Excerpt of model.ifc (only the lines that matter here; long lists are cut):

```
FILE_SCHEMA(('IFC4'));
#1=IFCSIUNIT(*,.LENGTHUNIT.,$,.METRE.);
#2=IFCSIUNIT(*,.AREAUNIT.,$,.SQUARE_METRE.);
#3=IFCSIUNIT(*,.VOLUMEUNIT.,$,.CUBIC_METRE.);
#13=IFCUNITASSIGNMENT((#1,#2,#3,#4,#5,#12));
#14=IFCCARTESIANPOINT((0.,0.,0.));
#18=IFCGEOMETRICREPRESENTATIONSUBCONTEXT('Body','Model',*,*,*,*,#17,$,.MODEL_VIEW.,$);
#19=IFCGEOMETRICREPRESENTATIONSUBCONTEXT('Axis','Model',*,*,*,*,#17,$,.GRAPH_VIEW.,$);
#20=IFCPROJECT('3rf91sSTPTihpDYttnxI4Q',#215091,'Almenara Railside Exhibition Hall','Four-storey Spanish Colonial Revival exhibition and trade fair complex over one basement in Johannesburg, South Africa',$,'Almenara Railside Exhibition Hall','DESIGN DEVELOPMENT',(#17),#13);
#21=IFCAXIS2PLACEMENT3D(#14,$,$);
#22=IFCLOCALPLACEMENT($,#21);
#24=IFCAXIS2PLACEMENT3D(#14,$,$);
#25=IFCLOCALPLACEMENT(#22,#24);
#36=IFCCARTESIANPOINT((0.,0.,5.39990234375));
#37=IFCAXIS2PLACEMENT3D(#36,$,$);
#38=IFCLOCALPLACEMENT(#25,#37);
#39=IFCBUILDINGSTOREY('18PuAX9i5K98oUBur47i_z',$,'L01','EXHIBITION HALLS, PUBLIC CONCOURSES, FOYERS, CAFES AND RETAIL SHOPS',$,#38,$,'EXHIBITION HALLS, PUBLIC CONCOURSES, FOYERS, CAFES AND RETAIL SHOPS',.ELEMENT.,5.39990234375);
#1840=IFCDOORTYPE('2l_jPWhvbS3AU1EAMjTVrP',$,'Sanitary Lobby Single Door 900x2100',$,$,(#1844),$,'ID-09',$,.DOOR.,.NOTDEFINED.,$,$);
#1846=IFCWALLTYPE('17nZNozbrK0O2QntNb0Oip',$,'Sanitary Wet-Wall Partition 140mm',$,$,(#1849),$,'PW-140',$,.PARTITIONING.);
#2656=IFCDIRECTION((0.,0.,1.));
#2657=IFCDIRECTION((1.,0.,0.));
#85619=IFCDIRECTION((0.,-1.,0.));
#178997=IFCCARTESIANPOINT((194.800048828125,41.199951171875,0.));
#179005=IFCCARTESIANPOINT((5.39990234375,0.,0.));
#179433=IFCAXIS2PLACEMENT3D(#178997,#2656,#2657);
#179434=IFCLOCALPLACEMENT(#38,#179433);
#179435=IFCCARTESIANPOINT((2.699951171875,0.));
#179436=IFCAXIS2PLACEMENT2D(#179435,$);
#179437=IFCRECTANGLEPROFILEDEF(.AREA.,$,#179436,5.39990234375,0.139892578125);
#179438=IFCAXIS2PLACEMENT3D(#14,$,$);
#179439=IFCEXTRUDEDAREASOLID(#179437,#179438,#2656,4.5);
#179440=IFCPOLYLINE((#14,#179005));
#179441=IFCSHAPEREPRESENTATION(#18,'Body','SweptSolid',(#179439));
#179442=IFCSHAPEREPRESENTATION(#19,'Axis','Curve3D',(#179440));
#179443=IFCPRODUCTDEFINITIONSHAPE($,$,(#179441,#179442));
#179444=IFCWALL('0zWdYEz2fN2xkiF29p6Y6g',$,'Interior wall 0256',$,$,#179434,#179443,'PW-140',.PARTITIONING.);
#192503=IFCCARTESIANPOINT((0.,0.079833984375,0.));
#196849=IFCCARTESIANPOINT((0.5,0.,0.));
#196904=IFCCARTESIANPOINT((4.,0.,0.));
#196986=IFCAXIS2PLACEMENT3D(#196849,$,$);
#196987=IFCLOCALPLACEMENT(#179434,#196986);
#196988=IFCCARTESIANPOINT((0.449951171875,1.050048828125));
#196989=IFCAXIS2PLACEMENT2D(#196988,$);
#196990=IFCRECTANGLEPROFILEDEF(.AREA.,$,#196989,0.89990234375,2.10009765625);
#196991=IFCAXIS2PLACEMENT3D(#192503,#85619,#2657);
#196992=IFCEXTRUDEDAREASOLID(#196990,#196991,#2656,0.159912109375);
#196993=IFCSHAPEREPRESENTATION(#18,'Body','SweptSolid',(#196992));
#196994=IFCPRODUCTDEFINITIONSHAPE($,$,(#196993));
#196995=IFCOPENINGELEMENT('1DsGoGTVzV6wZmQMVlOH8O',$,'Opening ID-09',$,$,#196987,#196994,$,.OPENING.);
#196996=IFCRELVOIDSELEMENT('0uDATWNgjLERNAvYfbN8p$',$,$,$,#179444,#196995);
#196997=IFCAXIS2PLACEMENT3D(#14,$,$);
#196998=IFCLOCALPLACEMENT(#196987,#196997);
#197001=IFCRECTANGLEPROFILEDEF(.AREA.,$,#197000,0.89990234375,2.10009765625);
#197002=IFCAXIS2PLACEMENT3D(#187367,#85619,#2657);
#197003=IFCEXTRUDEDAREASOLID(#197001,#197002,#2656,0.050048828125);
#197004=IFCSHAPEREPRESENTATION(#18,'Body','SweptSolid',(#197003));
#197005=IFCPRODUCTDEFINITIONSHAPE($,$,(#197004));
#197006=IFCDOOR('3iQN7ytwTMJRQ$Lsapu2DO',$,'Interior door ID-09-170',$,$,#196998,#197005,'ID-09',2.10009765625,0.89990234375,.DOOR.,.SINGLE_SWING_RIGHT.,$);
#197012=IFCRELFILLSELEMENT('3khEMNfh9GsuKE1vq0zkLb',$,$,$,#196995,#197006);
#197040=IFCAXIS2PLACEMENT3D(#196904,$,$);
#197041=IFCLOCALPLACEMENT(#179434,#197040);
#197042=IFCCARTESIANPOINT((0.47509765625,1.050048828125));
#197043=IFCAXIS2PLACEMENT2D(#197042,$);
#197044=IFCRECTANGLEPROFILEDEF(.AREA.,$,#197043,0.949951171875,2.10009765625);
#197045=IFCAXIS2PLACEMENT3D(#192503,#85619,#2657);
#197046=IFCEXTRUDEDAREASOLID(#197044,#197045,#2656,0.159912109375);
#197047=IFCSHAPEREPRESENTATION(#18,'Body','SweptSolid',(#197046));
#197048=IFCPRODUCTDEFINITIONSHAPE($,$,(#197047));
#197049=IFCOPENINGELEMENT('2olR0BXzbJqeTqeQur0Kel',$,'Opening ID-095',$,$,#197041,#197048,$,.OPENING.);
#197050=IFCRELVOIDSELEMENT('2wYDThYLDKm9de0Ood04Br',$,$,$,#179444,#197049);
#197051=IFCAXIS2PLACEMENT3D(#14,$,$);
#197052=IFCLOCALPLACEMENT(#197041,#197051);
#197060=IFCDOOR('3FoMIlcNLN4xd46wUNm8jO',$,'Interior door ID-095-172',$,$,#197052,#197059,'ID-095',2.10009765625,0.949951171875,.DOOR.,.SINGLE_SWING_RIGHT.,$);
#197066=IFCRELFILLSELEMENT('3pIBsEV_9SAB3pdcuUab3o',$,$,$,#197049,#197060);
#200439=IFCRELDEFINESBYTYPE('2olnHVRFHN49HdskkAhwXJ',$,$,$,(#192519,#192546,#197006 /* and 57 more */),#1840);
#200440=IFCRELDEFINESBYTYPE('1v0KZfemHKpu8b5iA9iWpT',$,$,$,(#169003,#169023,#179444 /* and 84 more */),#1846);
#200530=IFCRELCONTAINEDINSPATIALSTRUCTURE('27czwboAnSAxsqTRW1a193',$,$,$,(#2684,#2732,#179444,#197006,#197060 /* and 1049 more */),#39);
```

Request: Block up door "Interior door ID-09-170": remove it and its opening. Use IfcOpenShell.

```python
import ifcopenshell
import ifcopenshell.api.feature
import ifcopenshell.api.root
import ifcopenshell.geom
import ifcopenshell.util.shape

model = ifcopenshell.open("model.ifc")
settings = ifcopenshell.geom.settings()


def volume(element):
    """Net volume in cubic metres, openings subtracted."""
    shape = ifcopenshell.geom.create_shape(settings, element)
    return ifcopenshell.util.shape.get_volume(shape.geometry)


door = model.by_guid("3iQN7ytwTMJRQ$Lsapu2DO")
opening = door.FillsVoids[0].RelatingOpeningElement
wall = opening.VoidsElements[0].RelatingBuildingElement
before = volume(wall)

ifcopenshell.api.root.remove_product(model, product=door)
ifcopenshell.api.feature.remove_feature(model, feature=opening)

after = volume(wall)

print(f"wall volume {before:.3f} -> {after:.3f} m3")

model.write("model_edited.ifc")
```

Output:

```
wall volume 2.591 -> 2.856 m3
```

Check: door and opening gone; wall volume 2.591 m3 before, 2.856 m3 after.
